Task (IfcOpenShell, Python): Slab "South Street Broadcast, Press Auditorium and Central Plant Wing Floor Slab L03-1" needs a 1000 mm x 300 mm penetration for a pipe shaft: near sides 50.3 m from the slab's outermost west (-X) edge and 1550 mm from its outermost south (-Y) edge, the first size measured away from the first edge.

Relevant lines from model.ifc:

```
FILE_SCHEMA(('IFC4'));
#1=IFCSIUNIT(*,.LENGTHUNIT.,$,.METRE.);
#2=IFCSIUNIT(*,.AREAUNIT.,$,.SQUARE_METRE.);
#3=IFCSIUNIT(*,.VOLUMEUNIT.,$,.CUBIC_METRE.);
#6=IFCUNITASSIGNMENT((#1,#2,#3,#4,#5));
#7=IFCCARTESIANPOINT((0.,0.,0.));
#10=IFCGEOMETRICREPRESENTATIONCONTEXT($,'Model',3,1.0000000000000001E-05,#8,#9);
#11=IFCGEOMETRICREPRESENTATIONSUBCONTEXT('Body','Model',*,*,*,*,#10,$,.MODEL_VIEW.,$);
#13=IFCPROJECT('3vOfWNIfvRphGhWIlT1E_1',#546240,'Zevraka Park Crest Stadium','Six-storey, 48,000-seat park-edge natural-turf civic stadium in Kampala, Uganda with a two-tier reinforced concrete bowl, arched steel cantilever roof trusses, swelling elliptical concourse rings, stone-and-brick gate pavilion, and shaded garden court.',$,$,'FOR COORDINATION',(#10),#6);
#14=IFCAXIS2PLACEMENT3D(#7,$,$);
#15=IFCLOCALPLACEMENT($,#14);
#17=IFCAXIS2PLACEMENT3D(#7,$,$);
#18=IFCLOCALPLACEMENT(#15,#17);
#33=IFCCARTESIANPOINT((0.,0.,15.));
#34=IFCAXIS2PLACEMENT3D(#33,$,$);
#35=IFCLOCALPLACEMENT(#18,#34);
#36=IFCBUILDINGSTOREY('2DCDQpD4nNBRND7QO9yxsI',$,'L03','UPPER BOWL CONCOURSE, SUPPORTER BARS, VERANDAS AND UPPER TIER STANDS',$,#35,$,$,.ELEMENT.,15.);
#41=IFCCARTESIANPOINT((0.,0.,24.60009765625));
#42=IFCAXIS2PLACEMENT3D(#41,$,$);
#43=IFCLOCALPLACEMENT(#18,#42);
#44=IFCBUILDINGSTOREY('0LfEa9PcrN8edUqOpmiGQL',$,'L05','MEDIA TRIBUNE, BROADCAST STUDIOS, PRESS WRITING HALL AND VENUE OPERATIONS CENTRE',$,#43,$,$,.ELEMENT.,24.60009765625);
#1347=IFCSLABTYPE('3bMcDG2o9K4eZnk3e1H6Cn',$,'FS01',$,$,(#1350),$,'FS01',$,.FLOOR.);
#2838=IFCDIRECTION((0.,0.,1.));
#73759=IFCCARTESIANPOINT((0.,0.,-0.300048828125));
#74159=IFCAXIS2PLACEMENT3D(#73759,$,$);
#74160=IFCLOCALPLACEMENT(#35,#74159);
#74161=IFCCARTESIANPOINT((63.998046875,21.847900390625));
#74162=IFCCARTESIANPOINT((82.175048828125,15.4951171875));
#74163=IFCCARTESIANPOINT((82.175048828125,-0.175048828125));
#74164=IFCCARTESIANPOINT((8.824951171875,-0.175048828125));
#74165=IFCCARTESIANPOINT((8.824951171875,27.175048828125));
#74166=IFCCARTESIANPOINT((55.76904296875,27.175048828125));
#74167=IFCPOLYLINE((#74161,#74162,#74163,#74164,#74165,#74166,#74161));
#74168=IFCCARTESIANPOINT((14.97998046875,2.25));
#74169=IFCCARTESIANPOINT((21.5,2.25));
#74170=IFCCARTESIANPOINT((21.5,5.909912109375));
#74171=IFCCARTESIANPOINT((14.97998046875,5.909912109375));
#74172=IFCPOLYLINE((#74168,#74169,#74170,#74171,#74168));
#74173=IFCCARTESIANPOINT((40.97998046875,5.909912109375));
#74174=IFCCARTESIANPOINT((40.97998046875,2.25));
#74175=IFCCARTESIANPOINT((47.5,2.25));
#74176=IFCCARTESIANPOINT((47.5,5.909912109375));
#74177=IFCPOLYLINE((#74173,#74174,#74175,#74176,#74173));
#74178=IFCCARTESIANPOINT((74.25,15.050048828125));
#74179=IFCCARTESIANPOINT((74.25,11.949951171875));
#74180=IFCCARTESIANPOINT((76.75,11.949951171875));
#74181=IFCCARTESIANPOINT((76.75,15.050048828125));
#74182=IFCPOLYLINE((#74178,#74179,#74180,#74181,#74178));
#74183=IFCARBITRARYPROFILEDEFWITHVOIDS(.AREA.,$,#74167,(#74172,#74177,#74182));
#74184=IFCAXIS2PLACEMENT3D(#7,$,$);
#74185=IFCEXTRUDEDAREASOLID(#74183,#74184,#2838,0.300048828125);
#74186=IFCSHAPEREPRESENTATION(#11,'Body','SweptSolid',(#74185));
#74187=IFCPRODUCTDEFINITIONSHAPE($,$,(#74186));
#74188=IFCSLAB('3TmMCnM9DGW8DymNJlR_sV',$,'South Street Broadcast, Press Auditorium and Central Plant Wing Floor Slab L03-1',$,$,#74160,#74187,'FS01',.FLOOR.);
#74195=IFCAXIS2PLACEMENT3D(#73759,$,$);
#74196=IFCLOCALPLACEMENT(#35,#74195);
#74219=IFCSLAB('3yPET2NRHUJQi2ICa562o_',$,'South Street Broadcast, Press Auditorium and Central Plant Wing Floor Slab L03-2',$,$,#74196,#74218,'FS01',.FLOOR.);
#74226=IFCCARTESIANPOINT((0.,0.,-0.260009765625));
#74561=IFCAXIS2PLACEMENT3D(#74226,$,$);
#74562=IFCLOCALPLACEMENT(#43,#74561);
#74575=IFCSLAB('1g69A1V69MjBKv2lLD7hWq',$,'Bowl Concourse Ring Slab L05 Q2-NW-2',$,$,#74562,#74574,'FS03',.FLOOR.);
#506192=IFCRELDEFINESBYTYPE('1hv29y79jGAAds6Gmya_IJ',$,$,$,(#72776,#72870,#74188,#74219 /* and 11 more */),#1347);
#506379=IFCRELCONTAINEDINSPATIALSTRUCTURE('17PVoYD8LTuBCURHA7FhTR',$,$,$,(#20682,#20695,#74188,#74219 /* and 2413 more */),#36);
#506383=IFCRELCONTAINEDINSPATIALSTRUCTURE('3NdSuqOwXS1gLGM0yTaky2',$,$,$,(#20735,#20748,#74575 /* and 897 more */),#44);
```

```python
import numpy as np
import ifcopenshell
import ifcopenshell.api.feature
import ifcopenshell.api.geometry
import ifcopenshell.api.root
import ifcopenshell.geom
import ifcopenshell.util.placement
import ifcopenshell.util.representation
import ifcopenshell.util.shape
import ifcopenshell.util.unit

model = ifcopenshell.open("model.ifc")
unit_scale = ifcopenshell.util.unit.calculate_unit_scale(model)
settings = ifcopenshell.geom.settings()


def volume(element):
    """Net volume in cubic metres, openings subtracted."""
    shape = ifcopenshell.geom.create_shape(settings, element)
    return ifcopenshell.util.shape.get_volume(shape.geometry)


slab = model.by_guid("3TmMCnM9DGW8DymNJlR_sV")
before = volume(slab)

# Extent in the slab's own axes, in metres. The edges named are its -X and -Y sides.
slab_shape = ifcopenshell.geom.create_shape(settings, slab)
vertices = ifcopenshell.util.shape.get_vertices(slab_shape.geometry)
x_min, y_min, bottom = vertices.min(axis=0)
top = vertices[:, 2].max()

opening = ifcopenshell.api.root.create_entity(model, ifc_class="IfcOpeningElement", name="Pipe shaft opening", predefined_type="OPENING")
context = ifcopenshell.util.representation.get_context(model, "Model", "Body", "MODEL_VIEW")
width, depth = 1, 0.3
outline = [(0.0, 0.0), (width, 0.0), (width, depth), (0.0, depth), (0.0, 0.0)]
# Overshoot both faces by 50 mm so the cut is clean.
shape = ifcopenshell.api.geometry.add_slab_representation(
    model, context=context, depth=top - bottom + 0.1, polyline=outline
)
ifcopenshell.api.geometry.assign_representation(model, product=opening, representation=shape)

matrix = ifcopenshell.util.placement.get_local_placement(slab.ObjectPlacement)
matrix[:, 3] = matrix @ np.append(np.array([x_min + 50.3, y_min + 1.55, bottom - 0.05]) / unit_scale, 1.0)
ifcopenshell.api.geometry.edit_object_placement(model, product=opening, matrix=matrix, is_si=False)
ifcopenshell.api.feature.add_feature(model, feature=opening, element=slab)

after = volume(slab)

print(f"slab volume {before:.3f} -> {after:.3f} m3")

model.write("model-out.ifc")
```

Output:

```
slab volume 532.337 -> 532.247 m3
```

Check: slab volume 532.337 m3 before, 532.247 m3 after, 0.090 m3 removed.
